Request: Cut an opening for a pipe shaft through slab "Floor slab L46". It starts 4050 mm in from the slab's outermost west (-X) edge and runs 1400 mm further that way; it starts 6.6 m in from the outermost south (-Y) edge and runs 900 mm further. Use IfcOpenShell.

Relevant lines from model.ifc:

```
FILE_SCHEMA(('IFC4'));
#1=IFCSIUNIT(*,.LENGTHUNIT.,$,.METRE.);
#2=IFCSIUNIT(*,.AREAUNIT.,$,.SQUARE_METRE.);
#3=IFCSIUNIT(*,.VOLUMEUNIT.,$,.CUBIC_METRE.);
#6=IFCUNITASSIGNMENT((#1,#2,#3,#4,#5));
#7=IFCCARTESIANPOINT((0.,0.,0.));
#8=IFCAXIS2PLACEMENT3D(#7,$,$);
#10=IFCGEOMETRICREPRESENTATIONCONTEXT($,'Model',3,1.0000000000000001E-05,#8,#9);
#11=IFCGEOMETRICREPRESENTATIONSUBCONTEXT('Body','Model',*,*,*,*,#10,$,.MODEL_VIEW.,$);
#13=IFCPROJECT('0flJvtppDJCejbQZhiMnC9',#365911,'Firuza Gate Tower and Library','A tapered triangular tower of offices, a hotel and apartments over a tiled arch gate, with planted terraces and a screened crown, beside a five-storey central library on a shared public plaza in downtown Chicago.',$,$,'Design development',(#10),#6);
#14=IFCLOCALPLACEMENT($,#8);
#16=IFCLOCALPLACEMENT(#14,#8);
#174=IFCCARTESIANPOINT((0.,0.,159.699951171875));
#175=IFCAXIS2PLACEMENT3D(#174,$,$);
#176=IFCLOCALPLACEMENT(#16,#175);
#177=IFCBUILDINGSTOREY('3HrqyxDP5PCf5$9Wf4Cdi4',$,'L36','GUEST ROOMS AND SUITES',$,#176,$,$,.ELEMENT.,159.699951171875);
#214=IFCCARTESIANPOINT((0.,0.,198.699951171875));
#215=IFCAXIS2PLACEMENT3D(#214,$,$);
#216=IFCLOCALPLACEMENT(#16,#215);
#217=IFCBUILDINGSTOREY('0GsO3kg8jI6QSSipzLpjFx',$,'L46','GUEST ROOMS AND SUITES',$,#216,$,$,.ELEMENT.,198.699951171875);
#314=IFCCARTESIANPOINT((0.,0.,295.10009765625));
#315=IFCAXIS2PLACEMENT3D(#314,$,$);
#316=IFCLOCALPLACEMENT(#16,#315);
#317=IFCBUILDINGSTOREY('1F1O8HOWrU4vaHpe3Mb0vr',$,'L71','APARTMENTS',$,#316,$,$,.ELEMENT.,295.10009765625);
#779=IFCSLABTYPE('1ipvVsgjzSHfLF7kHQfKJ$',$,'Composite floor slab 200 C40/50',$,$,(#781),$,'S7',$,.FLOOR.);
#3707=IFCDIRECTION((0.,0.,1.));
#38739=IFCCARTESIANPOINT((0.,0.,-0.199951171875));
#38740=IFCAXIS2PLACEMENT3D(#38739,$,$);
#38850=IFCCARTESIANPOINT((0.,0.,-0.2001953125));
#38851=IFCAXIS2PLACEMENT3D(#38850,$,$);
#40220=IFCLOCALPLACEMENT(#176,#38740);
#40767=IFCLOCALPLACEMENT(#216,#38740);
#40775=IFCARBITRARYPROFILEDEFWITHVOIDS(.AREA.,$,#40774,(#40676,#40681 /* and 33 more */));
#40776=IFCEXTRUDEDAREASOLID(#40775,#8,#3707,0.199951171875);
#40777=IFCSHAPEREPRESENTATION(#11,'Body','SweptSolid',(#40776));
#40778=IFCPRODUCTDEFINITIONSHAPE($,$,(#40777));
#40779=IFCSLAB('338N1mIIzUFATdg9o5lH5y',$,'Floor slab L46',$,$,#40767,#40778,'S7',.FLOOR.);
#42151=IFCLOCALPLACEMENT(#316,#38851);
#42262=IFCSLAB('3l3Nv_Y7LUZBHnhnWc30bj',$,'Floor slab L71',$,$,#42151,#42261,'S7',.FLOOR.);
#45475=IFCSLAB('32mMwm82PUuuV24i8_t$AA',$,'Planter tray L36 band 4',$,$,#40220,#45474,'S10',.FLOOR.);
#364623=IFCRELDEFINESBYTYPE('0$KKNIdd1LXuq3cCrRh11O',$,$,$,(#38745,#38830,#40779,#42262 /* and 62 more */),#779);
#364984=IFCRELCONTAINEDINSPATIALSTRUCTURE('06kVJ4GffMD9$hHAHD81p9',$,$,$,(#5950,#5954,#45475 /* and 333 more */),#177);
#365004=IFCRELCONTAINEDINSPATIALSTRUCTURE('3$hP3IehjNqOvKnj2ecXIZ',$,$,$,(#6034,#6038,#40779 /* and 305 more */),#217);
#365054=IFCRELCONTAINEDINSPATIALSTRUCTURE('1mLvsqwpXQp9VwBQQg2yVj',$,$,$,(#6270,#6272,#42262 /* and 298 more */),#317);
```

```python
import numpy as np
import ifcopenshell
import ifcopenshell.api.feature
import ifcopenshell.api.geometry
import ifcopenshell.api.root
import ifcopenshell.geom
import ifcopenshell.util.placement
import ifcopenshell.util.representation
import ifcopenshell.util.shape
import ifcopenshell.util.unit

model = ifcopenshell.open("model.ifc")
unit_scale = ifcopenshell.util.unit.calculate_unit_scale(model)
settings = ifcopenshell.geom.settings()


def volume(element):
    """Net volume in cubic metres, openings subtracted."""
    shape = ifcopenshell.geom.create_shape(settings, element)
    return ifcopenshell.util.shape.get_volume(shape.geometry)


slab = model.by_id(40779)
before = volume(slab)

# Extent in the slab's own axes, in metres. The edges named are its -X and -Y sides.
slab_shape = ifcopenshell.geom.create_shape(settings, slab)
vertices = ifcopenshell.util.shape.get_vertices(slab_shape.geometry)
x_min, y_min, bottom = vertices.min(axis=0)
top = vertices[:, 2].max()

opening = ifcopenshell.api.root.create_entity(model, ifc_class="IfcOpeningElement", name="Pipe shaft opening", predefined_type="OPENING")
context = ifcopenshell.util.representation.get_context(model, "Model", "Body", "MODEL_VIEW")
width, depth = 1.4, 0.9
outline = [(0.0, 0.0), (width, 0.0), (width, depth), (0.0, depth), (0.0, 0.0)]
# Overshoot both faces by 50 mm so the cut is clean.
shape = ifcopenshell.api.geometry.add_slab_representation(
    model, context=context, depth=top - bottom + 0.1, polyline=outline
)
ifcopenshell.api.geometry.assign_representation(model, product=opening, representation=shape)

matrix = ifcopenshell.util.placement.get_local_placement(slab.ObjectPlacement)
matrix[:, 3] = matrix @ np.append(np.array([x_min + 4.05, y_min + 6.6, bottom - 0.05]) / unit_scale, 1.0)
ifcopenshell.api.geometry.edit_object_placement(model, product=opening, matrix=matrix, is_si=False)
ifcopenshell.api.feature.add_feature(model, feature=opening, element=slab)

after = volume(slab)

print(f"slab volume {before:.3f} -> {after:.3f} m3")

model.write("model_edited.ifc")
```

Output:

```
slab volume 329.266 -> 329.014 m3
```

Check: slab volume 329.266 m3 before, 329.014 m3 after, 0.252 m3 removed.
